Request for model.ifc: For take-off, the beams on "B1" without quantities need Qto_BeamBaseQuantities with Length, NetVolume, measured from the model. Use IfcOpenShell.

First a look at what the model holds.

```python
import ifcopenshell
import ifcopenshell.util.element
import ifcopenshell.util.unit

model = ifcopenshell.open("model.ifc")
print(model.schema)
for unit_type in ("LENGTHUNIT", "AREAUNIT", "VOLUMEUNIT"):
    print(unit_type, ifcopenshell.util.unit.calculate_unit_scale(model, unit_type))
storey = next(s for s in model.by_type("IfcBuildingStorey") if s.Name == "B1")
beams = [e for e in ifcopenshell.util.element.get_decomposition(storey) if e.is_a("IfcBeam")]
for e in sorted(beams, key=lambda e: e.id()):
    print(e.id(), e.is_a(), e.Name, list(ifcopenshell.util.element.get_psets(e, qtos_only=True)), sep=" | ")
```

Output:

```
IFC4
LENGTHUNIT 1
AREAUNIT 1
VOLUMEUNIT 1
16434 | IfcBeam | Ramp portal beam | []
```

```python
import ifcopenshell
import ifcopenshell.api.pset
import ifcopenshell.geom
import ifcopenshell.util.element
import ifcopenshell.util.shape
import ifcopenshell.util.unit

model = ifcopenshell.open("model.ifc")
unit_scale = ifcopenshell.util.unit.calculate_unit_scale(model)
volume_scale = ifcopenshell.util.unit.calculate_unit_scale(model, "VOLUMEUNIT")
settings = ifcopenshell.geom.settings()

storey = next(s for s in model.by_type("IfcBuildingStorey") if s.Name == "B1")
beams = [e for e in ifcopenshell.util.element.get_decomposition(storey) if e.is_a("IfcBeam")]

for e in sorted(beams, key=lambda e: e.id()):
    if ifcopenshell.util.element.get_psets(e, qtos_only=True, should_inherit=False):
        continue
    # Geometry comes back in metres, in the element's own axes.
    shape = ifcopenshell.geom.create_shape(settings, e)
    values = {
        "Length": ifcopenshell.util.shape.get_max_xyz(shape.geometry) / unit_scale,
        "NetVolume": ifcopenshell.util.shape.get_volume(shape.geometry) / volume_scale,
    }
    qto = ifcopenshell.api.pset.add_qto(model, product=e, name="Qto_BeamBaseQuantities")
    ifcopenshell.api.pset.edit_qto(model, qto=qto, properties=values)
    print(e.id(), {k: round(v, 3) for k, v in values.items()})

model.write("model_rev.ifc")
```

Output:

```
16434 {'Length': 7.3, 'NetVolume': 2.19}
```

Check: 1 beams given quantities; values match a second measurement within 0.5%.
